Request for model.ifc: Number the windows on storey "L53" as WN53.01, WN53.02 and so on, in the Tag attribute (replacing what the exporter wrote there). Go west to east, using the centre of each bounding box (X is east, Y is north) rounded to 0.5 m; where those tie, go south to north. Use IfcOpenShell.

First a look at what the model holds.

```python
import ifcopenshell
import ifcopenshell.util.element
import ifcopenshell.util.placement

model = ifcopenshell.open("model.ifc")
print(model.schema)
storey = next(s for s in model.by_type("IfcBuildingStorey") if s.Name == "L53")
windows = [e for e in ifcopenshell.util.element.get_decomposition(storey) if e.is_a("IfcWindow")]
for e in sorted(windows, key=lambda e: e.id()):
    origin = ifcopenshell.util.placement.get_local_placement(e.ObjectPlacement)[:3, 3]
    print(e.id(), e.Tag, e.Name, origin.round(2) + 0.0, sep=" | ")
```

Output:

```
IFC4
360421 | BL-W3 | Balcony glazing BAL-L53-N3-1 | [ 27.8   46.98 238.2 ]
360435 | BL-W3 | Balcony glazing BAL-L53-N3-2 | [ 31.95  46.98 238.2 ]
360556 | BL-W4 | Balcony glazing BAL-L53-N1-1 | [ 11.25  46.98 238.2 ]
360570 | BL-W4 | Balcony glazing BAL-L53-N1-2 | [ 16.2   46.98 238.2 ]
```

```python
import ifcopenshell
import ifcopenshell.geom
import ifcopenshell.util.element
import ifcopenshell.util.shape

model = ifcopenshell.open("model.ifc")
settings = ifcopenshell.geom.settings()
settings.set("use-world-coords", True)


def centre(element):
    shape = ifcopenshell.geom.create_shape(settings, element)
    return ifcopenshell.util.shape.get_bbox_centroid(shape.geometry)


storey = next(s for s in model.by_type("IfcBuildingStorey") if s.Name == "L53")
windows = [e for e in ifcopenshell.util.element.get_decomposition(storey) if e.is_a("IfcWindow")]

# Insertion points can sit at a corner or the storey origin, so sort by the geometry (in metres).
centres = {e: centre(e) for e in windows}
windows.sort(key=lambda e: (round(centres[e][0] / 0.5), centres[e][1]))

for i, e in enumerate(windows, start=1):
    number = f"WN53.{i:02d}"
    e.Tag = number
    print(e.id(), number)

model.write("model_edited.ifc")
```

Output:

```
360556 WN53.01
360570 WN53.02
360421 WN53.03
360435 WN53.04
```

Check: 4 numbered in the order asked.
